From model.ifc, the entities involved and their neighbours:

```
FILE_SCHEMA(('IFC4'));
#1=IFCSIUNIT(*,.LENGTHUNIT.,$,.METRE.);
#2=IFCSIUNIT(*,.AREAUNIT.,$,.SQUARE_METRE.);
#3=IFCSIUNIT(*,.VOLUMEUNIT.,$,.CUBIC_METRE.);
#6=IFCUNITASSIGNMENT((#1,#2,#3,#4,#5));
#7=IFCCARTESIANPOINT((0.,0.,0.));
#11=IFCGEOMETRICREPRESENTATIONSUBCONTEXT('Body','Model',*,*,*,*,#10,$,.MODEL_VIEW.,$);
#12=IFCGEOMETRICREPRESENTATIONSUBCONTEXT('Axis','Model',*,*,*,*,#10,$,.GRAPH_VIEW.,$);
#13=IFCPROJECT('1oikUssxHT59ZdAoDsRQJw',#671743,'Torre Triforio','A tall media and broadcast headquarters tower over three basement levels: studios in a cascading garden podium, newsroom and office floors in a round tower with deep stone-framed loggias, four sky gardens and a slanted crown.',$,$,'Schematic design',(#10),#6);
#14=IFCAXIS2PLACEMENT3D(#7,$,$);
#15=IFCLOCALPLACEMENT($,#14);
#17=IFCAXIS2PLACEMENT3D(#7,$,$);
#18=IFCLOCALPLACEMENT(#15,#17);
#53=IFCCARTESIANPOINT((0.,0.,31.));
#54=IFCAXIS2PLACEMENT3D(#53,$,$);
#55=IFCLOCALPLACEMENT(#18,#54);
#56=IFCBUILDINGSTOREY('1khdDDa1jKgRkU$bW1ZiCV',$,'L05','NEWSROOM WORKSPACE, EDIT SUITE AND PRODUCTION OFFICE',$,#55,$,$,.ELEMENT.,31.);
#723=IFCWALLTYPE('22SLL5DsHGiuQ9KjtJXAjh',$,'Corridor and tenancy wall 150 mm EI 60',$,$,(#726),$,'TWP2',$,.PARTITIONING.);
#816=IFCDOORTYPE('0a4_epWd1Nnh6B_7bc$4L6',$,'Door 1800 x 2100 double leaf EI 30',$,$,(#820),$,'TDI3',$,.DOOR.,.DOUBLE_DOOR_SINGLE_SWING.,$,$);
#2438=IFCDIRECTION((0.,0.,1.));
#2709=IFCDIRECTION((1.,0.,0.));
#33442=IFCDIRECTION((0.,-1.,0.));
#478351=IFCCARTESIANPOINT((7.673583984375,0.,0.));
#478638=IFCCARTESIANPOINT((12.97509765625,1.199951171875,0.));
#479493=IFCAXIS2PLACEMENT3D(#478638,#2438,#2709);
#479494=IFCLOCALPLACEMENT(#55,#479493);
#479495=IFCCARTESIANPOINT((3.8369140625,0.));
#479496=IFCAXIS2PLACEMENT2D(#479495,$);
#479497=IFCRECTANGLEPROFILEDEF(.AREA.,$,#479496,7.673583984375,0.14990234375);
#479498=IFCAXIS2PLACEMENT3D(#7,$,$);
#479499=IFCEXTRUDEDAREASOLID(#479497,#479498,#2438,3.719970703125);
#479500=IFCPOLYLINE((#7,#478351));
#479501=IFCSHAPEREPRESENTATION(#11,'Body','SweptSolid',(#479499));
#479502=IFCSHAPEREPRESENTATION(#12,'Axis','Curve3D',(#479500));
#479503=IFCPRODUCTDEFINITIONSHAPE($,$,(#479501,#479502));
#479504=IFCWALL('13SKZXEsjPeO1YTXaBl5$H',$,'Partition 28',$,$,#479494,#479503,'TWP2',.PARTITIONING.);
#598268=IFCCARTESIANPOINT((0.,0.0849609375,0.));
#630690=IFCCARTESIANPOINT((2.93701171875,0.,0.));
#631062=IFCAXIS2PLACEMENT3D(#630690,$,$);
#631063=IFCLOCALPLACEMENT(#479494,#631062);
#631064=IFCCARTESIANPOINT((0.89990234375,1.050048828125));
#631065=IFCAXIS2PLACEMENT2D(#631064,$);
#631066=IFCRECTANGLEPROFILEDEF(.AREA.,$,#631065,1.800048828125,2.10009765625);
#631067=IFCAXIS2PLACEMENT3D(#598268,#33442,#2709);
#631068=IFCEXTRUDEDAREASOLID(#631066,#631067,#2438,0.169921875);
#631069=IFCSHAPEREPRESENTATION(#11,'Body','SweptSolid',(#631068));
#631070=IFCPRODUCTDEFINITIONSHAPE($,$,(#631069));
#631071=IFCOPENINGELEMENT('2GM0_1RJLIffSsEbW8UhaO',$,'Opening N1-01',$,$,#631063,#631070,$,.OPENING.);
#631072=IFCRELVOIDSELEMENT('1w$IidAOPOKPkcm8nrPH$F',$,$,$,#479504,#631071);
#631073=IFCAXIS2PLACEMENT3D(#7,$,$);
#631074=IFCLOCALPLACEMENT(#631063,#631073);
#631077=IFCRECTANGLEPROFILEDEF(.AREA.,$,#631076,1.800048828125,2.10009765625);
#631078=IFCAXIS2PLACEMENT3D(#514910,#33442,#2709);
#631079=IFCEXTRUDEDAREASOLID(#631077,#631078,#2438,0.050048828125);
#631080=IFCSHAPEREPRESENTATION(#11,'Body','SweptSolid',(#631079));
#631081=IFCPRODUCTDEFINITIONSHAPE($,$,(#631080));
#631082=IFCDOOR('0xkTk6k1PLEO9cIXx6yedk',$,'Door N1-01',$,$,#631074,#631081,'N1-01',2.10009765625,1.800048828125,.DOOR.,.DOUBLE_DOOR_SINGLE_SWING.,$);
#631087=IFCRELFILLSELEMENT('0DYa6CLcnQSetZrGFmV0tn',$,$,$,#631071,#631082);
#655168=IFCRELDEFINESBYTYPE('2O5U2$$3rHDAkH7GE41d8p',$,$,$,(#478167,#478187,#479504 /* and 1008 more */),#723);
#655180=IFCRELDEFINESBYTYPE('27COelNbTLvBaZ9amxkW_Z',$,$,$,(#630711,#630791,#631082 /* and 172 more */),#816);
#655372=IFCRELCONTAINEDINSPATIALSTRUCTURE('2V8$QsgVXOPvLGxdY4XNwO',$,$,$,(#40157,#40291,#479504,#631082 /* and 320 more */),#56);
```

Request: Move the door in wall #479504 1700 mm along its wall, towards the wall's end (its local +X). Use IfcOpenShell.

```python
import ifcopenshell
import ifcopenshell.api.geometry
import ifcopenshell.util.placement
import ifcopenshell.util.unit

model = ifcopenshell.open("model.ifc")
unit_scale = ifcopenshell.util.unit.calculate_unit_scale(model)

door = model.by_guid("0xkTk6k1PLEO9cIXx6yedk")
opening = door.FillsVoids[0].RelatingOpeningElement
wall = opening.VoidsElements[0].RelatingBuildingElement

wall_matrix = ifcopenshell.util.placement.get_local_placement(wall.ObjectPlacement)
shift = wall_matrix[:3, 0] * 1.7 / unit_scale
before = ifcopenshell.util.placement.get_local_placement(door.ObjectPlacement)[:3, 3].copy()

# The door is placed relative to its opening, so it follows when the opening moves.
matrix = ifcopenshell.util.placement.get_local_placement(opening.ObjectPlacement)
matrix[:3, 3] += shift
ifcopenshell.api.geometry.edit_object_placement(
    model, product=opening, matrix=matrix, is_si=False, should_transform_children=True
)

after = ifcopenshell.util.placement.get_local_placement(door.ObjectPlacement)[:3, 3]
print("door moved by", (after - before).round(3) + 0.0)

model.write("model_rev.ifc")
```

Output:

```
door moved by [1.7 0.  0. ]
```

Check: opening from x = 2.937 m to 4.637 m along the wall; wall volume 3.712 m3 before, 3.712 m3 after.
